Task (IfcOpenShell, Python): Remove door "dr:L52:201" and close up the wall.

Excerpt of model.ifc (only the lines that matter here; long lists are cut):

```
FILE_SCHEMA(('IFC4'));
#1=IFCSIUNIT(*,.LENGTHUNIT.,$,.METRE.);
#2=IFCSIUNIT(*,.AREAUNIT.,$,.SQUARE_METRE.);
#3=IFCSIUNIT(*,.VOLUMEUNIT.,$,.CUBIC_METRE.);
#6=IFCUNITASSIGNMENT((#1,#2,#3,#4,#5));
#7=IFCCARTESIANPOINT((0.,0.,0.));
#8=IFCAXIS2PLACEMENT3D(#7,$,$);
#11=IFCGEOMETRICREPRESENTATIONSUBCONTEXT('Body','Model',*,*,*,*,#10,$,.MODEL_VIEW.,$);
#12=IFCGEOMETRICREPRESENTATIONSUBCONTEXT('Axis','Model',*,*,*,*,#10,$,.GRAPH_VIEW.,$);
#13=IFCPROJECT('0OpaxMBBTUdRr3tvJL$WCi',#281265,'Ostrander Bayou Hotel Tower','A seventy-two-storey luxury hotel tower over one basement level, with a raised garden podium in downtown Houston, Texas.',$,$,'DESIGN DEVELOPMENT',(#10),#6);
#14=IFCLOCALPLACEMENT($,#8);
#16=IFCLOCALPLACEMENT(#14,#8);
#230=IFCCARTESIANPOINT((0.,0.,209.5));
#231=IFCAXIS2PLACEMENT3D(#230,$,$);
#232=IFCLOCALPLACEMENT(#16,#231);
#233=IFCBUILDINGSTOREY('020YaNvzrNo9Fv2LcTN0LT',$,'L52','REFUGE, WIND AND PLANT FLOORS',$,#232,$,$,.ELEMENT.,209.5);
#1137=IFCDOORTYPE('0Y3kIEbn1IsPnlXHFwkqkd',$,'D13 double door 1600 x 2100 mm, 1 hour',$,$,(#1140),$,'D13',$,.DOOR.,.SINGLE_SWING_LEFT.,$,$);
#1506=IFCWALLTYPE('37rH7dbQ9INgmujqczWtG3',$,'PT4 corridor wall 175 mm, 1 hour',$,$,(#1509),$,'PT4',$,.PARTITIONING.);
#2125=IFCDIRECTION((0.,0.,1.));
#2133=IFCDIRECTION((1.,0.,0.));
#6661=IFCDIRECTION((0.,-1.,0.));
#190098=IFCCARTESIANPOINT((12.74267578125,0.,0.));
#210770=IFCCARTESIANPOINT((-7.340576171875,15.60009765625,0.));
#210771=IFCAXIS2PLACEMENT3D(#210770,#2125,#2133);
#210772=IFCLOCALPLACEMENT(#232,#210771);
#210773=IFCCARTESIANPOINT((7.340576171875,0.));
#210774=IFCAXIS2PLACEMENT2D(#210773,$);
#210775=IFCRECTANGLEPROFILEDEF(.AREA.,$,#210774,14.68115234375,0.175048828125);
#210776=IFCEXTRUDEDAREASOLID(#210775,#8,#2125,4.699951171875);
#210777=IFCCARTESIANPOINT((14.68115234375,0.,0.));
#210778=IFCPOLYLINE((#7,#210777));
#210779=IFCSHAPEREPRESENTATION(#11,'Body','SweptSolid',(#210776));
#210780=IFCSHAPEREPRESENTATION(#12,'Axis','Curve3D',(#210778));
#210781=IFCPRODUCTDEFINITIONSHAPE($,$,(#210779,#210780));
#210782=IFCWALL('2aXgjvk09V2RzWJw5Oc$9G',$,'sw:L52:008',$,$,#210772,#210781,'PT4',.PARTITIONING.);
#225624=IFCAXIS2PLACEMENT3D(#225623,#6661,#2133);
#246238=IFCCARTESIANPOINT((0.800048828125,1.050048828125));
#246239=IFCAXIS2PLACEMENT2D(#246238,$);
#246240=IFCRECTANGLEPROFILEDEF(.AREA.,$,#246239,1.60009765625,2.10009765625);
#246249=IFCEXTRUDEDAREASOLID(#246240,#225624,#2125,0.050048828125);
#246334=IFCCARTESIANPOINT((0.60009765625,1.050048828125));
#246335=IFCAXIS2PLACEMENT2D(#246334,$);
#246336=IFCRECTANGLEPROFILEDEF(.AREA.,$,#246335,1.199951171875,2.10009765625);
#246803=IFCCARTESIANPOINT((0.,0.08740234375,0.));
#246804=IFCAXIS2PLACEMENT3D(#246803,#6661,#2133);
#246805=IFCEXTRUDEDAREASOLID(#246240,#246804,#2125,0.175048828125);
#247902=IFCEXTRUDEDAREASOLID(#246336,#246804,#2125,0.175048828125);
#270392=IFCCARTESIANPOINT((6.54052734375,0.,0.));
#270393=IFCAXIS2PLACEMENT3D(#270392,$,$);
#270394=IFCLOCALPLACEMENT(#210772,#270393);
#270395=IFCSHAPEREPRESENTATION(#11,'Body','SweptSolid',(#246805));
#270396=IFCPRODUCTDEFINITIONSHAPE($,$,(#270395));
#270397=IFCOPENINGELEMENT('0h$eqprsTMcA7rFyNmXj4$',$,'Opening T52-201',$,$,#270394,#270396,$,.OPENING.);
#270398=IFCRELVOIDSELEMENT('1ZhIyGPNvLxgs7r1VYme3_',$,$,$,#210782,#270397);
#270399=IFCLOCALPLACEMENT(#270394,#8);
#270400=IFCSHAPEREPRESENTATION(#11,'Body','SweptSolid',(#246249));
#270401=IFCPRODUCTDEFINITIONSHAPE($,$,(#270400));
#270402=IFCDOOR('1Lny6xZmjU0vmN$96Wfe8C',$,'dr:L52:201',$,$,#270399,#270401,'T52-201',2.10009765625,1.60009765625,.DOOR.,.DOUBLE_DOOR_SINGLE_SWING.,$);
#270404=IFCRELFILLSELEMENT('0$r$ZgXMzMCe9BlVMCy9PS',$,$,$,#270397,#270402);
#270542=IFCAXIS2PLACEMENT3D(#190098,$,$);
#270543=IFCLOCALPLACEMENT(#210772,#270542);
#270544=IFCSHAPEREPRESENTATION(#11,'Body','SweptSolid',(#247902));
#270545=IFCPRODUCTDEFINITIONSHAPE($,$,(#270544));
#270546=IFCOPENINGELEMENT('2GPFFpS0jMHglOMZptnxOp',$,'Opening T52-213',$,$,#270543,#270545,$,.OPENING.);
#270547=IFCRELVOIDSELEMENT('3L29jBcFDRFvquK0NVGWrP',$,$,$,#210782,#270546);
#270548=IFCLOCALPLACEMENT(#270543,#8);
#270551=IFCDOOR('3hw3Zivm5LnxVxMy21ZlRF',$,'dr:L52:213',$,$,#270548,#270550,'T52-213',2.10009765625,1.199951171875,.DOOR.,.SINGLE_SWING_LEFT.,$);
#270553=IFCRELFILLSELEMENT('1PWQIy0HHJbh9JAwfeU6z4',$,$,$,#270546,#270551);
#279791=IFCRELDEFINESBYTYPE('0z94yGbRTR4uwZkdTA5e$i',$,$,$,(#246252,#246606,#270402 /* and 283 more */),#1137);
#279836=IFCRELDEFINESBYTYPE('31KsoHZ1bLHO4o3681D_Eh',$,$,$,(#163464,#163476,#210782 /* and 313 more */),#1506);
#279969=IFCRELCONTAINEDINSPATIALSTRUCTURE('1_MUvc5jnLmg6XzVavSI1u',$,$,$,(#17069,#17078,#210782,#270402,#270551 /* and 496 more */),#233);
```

```python
import ifcopenshell
import ifcopenshell.api.feature
import ifcopenshell.api.root
import ifcopenshell.geom
import ifcopenshell.util.shape

model = ifcopenshell.open("model.ifc")
settings = ifcopenshell.geom.settings()


def volume(element):
    """Net volume in cubic metres, openings subtracted."""
    shape = ifcopenshell.geom.create_shape(settings, element)
    return ifcopenshell.util.shape.get_volume(shape.geometry)


door = model.by_id(270402)
opening = door.FillsVoids[0].RelatingOpeningElement
wall = opening.VoidsElements[0].RelatingBuildingElement
before = volume(wall)

ifcopenshell.api.root.remove_product(model, product=door)
ifcopenshell.api.feature.remove_feature(model, feature=opening)

after = volume(wall)

print(f"wall volume {before:.3f} -> {after:.3f} m3")

model.write("model_v2.ifc")
```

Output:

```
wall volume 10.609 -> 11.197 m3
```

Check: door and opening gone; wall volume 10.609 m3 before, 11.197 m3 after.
